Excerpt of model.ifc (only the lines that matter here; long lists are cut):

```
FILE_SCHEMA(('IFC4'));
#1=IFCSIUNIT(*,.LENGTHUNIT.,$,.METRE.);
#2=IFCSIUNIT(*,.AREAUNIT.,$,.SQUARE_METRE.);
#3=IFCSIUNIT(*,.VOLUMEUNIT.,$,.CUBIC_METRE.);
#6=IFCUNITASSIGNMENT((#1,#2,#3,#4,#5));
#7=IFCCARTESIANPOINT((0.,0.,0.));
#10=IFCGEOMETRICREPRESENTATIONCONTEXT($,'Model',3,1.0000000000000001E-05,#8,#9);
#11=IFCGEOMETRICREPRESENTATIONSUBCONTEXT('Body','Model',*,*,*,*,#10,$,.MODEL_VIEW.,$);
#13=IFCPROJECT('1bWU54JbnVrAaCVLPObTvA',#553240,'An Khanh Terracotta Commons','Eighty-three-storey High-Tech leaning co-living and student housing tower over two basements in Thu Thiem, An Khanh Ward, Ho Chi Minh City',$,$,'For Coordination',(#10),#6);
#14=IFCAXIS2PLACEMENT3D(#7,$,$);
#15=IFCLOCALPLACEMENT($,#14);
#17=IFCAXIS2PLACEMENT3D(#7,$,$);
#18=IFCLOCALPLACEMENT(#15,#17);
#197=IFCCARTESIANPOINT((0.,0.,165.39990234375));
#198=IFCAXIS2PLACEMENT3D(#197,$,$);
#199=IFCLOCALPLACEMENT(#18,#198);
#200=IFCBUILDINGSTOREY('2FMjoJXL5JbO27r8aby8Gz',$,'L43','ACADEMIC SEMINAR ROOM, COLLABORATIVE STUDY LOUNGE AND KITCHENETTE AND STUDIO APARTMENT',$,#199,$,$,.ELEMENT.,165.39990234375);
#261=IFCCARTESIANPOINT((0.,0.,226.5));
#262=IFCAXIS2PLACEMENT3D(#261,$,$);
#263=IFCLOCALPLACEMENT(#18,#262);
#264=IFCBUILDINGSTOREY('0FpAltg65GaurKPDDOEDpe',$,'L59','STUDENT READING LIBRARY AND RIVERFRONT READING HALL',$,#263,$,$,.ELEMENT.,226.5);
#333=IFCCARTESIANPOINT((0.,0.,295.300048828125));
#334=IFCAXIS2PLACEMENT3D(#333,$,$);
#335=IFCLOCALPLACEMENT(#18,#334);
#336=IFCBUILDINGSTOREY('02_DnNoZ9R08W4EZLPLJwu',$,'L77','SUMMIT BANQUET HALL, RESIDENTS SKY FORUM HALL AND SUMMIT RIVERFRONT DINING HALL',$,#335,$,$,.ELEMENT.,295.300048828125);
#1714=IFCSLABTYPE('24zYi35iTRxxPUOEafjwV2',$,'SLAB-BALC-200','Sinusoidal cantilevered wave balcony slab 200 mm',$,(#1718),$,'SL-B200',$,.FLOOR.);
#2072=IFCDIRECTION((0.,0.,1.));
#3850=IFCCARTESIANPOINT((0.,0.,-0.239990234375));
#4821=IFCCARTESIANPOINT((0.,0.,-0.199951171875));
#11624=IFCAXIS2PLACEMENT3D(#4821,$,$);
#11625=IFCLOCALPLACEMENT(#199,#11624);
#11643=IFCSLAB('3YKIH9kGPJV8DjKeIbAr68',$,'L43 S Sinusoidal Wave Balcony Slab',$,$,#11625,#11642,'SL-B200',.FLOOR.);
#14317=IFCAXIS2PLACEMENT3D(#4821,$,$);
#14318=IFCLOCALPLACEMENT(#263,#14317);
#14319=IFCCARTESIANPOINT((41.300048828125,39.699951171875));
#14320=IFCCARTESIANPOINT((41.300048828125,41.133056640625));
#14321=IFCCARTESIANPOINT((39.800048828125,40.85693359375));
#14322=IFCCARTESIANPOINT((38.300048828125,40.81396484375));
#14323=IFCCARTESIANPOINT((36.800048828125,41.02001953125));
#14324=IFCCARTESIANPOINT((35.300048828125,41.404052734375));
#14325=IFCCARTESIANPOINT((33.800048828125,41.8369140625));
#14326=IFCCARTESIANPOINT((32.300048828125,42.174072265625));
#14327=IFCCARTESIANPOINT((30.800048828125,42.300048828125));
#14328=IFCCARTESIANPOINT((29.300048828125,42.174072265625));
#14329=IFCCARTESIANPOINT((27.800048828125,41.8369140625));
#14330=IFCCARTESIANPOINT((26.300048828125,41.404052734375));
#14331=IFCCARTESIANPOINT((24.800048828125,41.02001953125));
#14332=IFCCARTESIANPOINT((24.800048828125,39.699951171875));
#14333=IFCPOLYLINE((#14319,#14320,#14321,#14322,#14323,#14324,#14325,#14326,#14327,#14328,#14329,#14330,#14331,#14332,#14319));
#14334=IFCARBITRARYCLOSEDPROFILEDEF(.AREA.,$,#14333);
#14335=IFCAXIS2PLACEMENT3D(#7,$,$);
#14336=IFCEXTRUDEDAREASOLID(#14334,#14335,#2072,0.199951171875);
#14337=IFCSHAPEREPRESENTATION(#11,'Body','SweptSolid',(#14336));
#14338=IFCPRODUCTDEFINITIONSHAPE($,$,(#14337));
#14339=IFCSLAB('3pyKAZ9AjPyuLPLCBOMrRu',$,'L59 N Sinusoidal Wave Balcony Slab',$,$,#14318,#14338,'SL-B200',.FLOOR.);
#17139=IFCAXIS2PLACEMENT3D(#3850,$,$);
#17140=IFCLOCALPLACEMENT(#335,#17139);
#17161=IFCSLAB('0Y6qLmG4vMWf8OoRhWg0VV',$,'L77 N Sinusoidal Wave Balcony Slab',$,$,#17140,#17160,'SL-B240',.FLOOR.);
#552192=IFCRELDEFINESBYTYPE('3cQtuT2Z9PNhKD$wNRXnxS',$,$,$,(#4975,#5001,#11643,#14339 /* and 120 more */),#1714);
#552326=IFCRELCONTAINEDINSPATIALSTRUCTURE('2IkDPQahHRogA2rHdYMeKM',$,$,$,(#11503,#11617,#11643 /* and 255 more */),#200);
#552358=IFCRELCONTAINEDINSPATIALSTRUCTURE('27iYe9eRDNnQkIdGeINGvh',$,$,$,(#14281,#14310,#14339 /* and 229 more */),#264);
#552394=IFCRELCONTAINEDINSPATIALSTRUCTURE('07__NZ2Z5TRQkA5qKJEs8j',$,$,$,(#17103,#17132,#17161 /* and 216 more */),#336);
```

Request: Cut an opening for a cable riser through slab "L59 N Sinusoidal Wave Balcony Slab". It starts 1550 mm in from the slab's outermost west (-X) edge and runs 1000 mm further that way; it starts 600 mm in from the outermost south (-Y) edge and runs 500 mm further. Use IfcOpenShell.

```python
import numpy as np
import ifcopenshell
import ifcopenshell.api.feature
import ifcopenshell.api.geometry
import ifcopenshell.api.root
import ifcopenshell.geom
import ifcopenshell.util.placement
import ifcopenshell.util.representation
import ifcopenshell.util.shape
import ifcopenshell.util.unit

model = ifcopenshell.open("model.ifc")
unit_scale = ifcopenshell.util.unit.calculate_unit_scale(model)
settings = ifcopenshell.geom.settings()


def volume(element):
    """Net volume in cubic metres, openings subtracted."""
    shape = ifcopenshell.geom.create_shape(settings, element)
    return ifcopenshell.util.shape.get_volume(shape.geometry)


slab = model.by_id(14339)
before = volume(slab)

# Extent in the slab's own axes, in metres. The edges named are its -X and -Y sides.
slab_shape = ifcopenshell.geom.create_shape(settings, slab)
vertices = ifcopenshell.util.shape.get_vertices(slab_shape.geometry)
x_min, y_min, bottom = vertices.min(axis=0)
top = vertices[:, 2].max()

opening = ifcopenshell.api.root.create_entity(model, ifc_class="IfcOpeningElement", name="Cable riser opening", predefined_type="OPENING")
context = ifcopenshell.util.representation.get_context(model, "Model", "Body", "MODEL_VIEW")
width, depth = 1, 0.5
outline = [(0.0, 0.0), (width, 0.0), (width, depth), (0.0, depth), (0.0, 0.0)]
# Overshoot both faces by 50 mm so the cut is clean.
shape = ifcopenshell.api.geometry.add_slab_representation(
    model, context=context, depth=top - bottom + 0.1, polyline=outline
)
ifcopenshell.api.geometry.assign_representation(model, product=opening, representation=shape)

matrix = ifcopenshell.util.placement.get_local_placement(slab.ObjectPlacement)
matrix[:, 3] = matrix @ np.append(np.array([x_min + 1.55, y_min + 0.6, bottom - 0.05]) / unit_scale, 1.0)
ifcopenshell.api.geometry.edit_object_placement(model, product=opening, matrix=matrix, is_si=False)
ifcopenshell.api.feature.add_feature(model, feature=opening, element=slab)

after = volume(slab)

print(f"slab volume {before:.3f} -> {after:.3f} m3")

model.write("model_updated.ifc")
```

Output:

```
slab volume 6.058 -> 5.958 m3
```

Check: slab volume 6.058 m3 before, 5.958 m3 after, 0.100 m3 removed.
